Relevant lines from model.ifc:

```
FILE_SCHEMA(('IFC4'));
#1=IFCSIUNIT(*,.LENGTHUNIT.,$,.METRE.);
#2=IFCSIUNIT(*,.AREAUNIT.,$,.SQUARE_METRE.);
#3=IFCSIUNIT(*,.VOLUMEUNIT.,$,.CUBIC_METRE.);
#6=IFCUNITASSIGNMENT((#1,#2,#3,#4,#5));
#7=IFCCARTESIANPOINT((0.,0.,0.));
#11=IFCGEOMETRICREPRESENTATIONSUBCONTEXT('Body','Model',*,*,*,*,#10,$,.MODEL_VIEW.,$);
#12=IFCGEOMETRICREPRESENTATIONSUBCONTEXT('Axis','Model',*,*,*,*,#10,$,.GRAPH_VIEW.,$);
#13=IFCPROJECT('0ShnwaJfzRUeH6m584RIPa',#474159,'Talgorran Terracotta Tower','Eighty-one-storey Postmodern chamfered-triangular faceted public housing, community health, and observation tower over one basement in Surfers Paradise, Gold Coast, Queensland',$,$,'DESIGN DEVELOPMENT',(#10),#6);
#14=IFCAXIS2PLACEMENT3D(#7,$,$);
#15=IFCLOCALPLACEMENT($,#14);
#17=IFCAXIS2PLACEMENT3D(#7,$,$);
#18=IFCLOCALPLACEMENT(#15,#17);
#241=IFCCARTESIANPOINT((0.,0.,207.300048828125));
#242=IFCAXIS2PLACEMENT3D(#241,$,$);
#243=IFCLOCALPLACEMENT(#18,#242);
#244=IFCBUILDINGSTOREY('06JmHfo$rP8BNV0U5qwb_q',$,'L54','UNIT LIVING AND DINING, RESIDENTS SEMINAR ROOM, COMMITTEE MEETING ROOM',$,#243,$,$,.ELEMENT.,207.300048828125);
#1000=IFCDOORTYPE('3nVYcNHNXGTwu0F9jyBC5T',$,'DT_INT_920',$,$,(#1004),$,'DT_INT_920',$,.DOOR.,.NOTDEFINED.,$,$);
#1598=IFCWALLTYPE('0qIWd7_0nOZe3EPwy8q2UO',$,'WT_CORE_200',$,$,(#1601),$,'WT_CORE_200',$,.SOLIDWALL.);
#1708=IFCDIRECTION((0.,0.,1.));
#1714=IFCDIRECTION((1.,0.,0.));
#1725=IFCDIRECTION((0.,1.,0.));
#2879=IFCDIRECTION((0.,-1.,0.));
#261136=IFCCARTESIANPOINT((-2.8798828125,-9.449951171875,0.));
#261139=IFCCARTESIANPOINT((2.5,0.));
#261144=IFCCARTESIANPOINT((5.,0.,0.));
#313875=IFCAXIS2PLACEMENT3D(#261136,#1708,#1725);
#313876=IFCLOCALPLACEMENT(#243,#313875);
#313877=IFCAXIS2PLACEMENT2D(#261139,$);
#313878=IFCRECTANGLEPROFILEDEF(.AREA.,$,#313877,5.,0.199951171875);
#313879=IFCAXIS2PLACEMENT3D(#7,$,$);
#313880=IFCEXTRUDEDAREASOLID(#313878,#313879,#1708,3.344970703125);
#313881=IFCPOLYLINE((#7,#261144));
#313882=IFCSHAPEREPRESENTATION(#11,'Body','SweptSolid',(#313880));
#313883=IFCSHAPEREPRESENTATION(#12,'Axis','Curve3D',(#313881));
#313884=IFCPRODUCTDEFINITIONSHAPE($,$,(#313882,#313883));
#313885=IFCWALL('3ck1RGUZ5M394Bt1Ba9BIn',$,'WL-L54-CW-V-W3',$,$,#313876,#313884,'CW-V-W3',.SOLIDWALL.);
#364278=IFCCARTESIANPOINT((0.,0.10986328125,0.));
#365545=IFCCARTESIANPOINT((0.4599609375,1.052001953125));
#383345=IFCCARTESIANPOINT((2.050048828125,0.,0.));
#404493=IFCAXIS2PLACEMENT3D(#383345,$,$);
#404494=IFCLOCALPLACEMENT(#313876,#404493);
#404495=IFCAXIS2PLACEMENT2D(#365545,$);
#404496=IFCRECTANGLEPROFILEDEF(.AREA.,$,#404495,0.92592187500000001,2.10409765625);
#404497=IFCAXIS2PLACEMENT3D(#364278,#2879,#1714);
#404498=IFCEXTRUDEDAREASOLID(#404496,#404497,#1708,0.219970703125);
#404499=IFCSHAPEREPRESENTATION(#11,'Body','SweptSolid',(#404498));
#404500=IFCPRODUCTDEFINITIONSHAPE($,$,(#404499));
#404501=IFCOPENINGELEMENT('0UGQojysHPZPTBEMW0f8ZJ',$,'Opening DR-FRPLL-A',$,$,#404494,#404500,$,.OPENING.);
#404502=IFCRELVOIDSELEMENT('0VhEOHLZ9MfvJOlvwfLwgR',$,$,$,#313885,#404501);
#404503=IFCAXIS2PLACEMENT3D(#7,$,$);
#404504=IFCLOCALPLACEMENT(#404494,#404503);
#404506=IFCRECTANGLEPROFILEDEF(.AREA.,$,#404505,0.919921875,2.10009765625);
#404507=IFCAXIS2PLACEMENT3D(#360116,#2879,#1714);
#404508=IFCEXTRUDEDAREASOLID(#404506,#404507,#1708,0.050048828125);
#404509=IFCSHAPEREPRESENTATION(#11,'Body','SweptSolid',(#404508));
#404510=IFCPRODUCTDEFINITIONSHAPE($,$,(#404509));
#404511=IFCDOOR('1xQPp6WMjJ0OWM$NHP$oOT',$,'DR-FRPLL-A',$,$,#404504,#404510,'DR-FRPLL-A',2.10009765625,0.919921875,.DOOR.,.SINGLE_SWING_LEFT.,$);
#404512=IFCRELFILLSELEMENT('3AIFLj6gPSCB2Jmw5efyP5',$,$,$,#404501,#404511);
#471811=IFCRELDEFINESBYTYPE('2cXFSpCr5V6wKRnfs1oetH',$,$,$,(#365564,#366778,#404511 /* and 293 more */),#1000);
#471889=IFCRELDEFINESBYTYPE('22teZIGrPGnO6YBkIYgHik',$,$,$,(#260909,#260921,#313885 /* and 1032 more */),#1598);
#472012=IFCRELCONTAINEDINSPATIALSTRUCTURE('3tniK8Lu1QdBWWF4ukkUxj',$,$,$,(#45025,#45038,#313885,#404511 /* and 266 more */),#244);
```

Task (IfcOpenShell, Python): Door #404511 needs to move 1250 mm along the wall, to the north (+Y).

```python
import ifcopenshell
import ifcopenshell.api.geometry
import ifcopenshell.util.placement
import ifcopenshell.util.unit

model = ifcopenshell.open("model.ifc")
unit_scale = ifcopenshell.util.unit.calculate_unit_scale(model)

door = model.by_guid("1xQPp6WMjJ0OWM$NHP$oOT")
opening = door.FillsVoids[0].RelatingOpeningElement
wall = opening.VoidsElements[0].RelatingBuildingElement

wall_matrix = ifcopenshell.util.placement.get_local_placement(wall.ObjectPlacement)
shift = wall_matrix[:3, 0] * 1.25 / unit_scale
before = ifcopenshell.util.placement.get_local_placement(door.ObjectPlacement)[:3, 3].copy()

# The door is placed relative to its opening, so it follows when the opening moves.
matrix = ifcopenshell.util.placement.get_local_placement(opening.ObjectPlacement)
matrix[:3, 3] += shift
ifcopenshell.api.geometry.edit_object_placement(
    model, product=opening, matrix=matrix, is_si=False, should_transform_children=True
)

after = ifcopenshell.util.placement.get_local_placement(door.ObjectPlacement)[:3, 3]
print("door moved by", (after - before).round(3) + 0.0)

model.write("model_edited.ifc")
```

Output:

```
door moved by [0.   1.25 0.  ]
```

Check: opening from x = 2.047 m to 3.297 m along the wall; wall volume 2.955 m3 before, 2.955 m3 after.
